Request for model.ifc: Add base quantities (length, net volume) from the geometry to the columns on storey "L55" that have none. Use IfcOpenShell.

First a look at what the model holds.

```python
import ifcopenshell
import ifcopenshell.util.element
import ifcopenshell.util.unit

model = ifcopenshell.open("model.ifc")
print(model.schema)
for unit_type in ("LENGTHUNIT", "AREAUNIT", "VOLUMEUNIT"):
    print(unit_type, ifcopenshell.util.unit.calculate_unit_scale(model, unit_type))
storey = next(s for s in model.by_type("IfcBuildingStorey") if s.Name == "L55")
columns = [e for e in ifcopenshell.util.element.get_decomposition(storey) if e.is_a("IfcColumn")]
for e in sorted(columns, key=lambda e: e.id()):
    print(e.id(), e.is_a(), e.Name, list(ifcopenshell.util.element.get_psets(e, qtos_only=True)), sep=" | ")
```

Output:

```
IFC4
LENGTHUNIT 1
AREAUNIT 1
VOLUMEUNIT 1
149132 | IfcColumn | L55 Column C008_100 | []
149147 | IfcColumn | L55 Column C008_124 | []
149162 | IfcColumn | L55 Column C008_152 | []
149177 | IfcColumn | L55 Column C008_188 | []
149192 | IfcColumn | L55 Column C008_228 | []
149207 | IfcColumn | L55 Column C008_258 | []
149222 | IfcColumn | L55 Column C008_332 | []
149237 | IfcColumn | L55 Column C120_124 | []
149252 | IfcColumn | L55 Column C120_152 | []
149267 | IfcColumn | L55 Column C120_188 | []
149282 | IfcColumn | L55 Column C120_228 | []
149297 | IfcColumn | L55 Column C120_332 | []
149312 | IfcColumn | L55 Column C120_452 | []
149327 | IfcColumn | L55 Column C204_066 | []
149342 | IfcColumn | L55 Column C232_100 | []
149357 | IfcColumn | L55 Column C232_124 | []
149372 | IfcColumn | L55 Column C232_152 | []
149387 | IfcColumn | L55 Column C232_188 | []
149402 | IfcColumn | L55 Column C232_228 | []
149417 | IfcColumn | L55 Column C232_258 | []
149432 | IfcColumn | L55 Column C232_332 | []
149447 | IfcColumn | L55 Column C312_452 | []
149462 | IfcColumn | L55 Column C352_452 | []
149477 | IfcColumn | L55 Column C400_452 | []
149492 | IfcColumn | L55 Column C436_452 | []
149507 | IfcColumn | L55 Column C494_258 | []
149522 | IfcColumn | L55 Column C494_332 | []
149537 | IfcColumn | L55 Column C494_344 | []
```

```python
import ifcopenshell
import ifcopenshell.api.pset
import ifcopenshell.geom
import ifcopenshell.util.element
import ifcopenshell.util.shape
import ifcopenshell.util.unit

model = ifcopenshell.open("model.ifc")
unit_scale = ifcopenshell.util.unit.calculate_unit_scale(model)
volume_scale = ifcopenshell.util.unit.calculate_unit_scale(model, "VOLUMEUNIT")
settings = ifcopenshell.geom.settings()

storey = next(s for s in model.by_type("IfcBuildingStorey") if s.Name == "L55")
columns = [e for e in ifcopenshell.util.element.get_decomposition(storey) if e.is_a("IfcColumn")]

for e in sorted(columns, key=lambda e: e.id()):
    if ifcopenshell.util.element.get_psets(e, qtos_only=True, should_inherit=False):
        continue
    # Geometry comes back in metres, in the element's own axes.
    shape = ifcopenshell.geom.create_shape(settings, e)
    values = {
        "Length": ifcopenshell.util.shape.get_z(shape.geometry) / unit_scale,
        "NetVolume": ifcopenshell.util.shape.get_volume(shape.geometry) / volume_scale,
    }
    qto = ifcopenshell.api.pset.add_qto(model, product=e, name="Qto_ColumnBaseQuantities")
    ifcopenshell.api.pset.edit_qto(model, qto=qto, properties=values)
    print(e.id(), {k: round(v, 3) for k, v in values.items()})

model.write("model-out.ifc")
```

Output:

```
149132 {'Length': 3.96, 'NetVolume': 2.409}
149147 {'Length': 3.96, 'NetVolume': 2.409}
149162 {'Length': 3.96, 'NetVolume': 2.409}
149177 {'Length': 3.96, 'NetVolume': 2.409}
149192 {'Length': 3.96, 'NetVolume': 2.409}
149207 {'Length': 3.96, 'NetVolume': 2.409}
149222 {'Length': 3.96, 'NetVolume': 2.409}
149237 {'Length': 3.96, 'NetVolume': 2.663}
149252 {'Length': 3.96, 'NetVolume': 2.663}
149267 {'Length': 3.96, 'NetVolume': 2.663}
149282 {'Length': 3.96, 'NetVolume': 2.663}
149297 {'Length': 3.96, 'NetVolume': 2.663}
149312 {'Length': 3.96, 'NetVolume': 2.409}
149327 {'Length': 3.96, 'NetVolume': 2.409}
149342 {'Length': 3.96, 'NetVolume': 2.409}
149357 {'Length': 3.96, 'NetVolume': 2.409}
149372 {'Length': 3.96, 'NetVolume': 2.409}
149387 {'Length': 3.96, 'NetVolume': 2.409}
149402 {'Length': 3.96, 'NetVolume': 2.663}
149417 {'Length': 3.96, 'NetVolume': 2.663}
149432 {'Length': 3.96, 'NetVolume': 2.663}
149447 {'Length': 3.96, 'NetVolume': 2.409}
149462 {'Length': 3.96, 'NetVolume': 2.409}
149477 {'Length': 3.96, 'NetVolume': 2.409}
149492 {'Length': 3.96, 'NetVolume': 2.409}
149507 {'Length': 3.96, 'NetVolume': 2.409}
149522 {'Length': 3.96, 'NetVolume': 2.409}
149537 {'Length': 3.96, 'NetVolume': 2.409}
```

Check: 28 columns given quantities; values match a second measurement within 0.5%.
